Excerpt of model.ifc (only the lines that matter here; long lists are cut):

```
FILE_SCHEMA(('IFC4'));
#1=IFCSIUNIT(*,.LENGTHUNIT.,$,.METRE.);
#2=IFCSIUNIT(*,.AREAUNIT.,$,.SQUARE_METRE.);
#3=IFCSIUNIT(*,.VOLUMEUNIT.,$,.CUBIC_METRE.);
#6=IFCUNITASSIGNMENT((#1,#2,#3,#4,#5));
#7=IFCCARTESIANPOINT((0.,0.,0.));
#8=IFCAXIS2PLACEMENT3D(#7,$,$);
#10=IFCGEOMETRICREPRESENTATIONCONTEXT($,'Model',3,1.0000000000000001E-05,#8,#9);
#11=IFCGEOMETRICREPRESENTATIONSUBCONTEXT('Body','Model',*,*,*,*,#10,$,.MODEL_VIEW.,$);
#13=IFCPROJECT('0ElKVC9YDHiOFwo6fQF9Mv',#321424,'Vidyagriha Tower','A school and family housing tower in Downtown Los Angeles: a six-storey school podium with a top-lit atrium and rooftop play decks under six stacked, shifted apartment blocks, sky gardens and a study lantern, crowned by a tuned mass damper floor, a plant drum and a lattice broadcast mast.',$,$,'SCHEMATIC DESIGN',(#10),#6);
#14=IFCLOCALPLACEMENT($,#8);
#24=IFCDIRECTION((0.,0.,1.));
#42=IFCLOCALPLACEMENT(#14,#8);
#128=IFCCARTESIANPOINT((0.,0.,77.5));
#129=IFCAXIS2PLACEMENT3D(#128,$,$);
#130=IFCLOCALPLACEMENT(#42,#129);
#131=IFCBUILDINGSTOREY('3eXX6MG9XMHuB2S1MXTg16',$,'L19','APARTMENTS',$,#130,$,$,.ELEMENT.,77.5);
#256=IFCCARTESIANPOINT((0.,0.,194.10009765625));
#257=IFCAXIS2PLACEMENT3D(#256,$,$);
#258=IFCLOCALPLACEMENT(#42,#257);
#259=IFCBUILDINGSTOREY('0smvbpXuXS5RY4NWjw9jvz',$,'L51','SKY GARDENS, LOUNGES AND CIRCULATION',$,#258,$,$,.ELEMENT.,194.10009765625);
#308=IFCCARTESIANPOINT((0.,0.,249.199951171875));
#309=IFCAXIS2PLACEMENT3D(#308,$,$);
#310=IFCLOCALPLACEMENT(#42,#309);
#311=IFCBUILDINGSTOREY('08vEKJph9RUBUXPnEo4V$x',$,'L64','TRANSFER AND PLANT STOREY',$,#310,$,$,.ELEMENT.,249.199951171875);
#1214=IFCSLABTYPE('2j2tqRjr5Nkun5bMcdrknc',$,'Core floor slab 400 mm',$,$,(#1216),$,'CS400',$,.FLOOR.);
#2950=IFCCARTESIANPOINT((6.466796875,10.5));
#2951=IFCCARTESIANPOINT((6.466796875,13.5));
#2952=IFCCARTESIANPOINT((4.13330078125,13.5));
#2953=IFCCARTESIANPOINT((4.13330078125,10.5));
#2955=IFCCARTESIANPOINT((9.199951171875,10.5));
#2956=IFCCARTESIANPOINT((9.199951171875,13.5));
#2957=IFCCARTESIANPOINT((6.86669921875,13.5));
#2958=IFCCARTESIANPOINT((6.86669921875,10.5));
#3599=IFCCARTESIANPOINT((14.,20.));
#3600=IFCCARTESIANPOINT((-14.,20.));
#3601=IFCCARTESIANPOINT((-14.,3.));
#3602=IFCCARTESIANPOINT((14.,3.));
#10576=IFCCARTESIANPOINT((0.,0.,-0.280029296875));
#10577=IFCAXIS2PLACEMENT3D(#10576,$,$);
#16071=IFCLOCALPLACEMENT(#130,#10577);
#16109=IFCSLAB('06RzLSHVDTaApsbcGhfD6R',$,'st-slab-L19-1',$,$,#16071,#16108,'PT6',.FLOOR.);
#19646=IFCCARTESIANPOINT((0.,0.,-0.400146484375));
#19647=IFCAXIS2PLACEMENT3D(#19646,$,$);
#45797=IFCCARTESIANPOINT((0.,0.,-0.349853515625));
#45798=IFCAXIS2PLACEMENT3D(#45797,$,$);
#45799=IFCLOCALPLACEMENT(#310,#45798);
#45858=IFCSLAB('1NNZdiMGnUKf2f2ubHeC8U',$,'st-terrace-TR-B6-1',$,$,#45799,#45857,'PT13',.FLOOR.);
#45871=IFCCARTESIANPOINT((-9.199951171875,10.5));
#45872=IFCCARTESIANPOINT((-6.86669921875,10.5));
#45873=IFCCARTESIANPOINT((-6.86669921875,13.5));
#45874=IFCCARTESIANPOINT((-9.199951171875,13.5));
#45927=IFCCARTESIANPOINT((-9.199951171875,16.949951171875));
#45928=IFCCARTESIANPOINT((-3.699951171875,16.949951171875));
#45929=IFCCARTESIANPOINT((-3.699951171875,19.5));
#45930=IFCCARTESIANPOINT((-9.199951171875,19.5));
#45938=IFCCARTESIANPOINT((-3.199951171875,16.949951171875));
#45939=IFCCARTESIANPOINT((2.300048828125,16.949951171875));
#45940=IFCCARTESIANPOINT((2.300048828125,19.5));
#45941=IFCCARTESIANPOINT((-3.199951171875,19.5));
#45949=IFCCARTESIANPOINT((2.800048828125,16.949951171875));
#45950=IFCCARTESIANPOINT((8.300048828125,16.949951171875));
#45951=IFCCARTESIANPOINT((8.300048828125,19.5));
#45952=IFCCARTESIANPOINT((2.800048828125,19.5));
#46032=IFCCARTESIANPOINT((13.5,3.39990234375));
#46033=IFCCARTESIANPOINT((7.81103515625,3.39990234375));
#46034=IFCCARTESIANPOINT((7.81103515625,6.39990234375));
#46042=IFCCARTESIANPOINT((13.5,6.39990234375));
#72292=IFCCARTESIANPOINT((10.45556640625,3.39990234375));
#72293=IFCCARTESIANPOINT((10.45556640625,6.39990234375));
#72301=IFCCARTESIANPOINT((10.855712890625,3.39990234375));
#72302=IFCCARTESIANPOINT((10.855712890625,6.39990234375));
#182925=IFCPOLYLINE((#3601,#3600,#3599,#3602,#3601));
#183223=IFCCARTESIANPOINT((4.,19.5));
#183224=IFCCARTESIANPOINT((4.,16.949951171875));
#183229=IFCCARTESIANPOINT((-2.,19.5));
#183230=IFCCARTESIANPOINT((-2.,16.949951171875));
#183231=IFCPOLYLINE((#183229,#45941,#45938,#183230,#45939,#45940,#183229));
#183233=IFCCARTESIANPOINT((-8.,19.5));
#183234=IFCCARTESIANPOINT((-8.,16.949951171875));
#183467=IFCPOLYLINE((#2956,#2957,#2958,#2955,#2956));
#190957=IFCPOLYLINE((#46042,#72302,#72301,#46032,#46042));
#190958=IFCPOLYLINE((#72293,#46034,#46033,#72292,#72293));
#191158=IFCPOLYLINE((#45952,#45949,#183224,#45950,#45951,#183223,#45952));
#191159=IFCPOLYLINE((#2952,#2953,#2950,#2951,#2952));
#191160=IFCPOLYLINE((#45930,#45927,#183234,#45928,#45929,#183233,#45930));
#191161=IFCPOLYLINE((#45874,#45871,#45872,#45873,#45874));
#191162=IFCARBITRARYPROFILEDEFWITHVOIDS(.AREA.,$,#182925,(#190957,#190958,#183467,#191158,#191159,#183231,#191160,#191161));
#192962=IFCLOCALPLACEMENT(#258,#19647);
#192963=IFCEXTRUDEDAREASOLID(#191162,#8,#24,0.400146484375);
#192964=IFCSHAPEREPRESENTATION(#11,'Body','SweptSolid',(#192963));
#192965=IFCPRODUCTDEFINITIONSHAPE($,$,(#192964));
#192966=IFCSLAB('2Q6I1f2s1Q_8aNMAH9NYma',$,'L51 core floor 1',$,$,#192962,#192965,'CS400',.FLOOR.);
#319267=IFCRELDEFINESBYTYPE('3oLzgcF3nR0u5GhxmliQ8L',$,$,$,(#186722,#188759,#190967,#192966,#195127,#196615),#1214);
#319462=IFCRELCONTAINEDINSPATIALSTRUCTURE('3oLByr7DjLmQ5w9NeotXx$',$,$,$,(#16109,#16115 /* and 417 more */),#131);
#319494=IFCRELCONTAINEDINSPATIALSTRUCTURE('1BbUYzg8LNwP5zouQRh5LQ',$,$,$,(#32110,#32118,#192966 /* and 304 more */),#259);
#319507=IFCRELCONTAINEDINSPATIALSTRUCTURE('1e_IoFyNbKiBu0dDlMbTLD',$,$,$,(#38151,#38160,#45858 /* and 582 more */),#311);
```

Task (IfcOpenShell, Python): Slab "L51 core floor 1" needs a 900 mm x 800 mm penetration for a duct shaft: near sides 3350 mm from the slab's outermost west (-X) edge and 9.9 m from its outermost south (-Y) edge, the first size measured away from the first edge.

```python
import numpy as np
import ifcopenshell
import ifcopenshell.api.feature
import ifcopenshell.api.geometry
import ifcopenshell.api.root
import ifcopenshell.geom
import ifcopenshell.util.placement
import ifcopenshell.util.representation
import ifcopenshell.util.shape
import ifcopenshell.util.unit

model = ifcopenshell.open("model.ifc")
unit_scale = ifcopenshell.util.unit.calculate_unit_scale(model)
settings = ifcopenshell.geom.settings()


def volume(element):
    """Net volume in cubic metres, openings subtracted."""
    shape = ifcopenshell.geom.create_shape(settings, element)
    return ifcopenshell.util.shape.get_volume(shape.geometry)


slab = model.by_id(192966)
before = volume(slab)

# Extent in the slab's own axes, in metres. The edges named are its -X and -Y sides.
slab_shape = ifcopenshell.geom.create_shape(settings, slab)
vertices = ifcopenshell.util.shape.get_vertices(slab_shape.geometry)
x_min, y_min, bottom = vertices.min(axis=0)
top = vertices[:, 2].max()

opening = ifcopenshell.api.root.create_entity(model, ifc_class="IfcOpeningElement", name="Duct shaft opening", predefined_type="OPENING")
context = ifcopenshell.util.representation.get_context(model, "Model", "Body", "MODEL_VIEW")
width, depth = 0.9, 0.8
outline = [(0.0, 0.0), (width, 0.0), (width, depth), (0.0, depth), (0.0, 0.0)]
# Overshoot both faces by 50 mm so the cut is clean.
shape = ifcopenshell.api.geometry.add_slab_representation(
    model, context=context, depth=top - bottom + 0.1, polyline=outline
)
ifcopenshell.api.geometry.assign_representation(model, product=opening, representation=shape)

matrix = ifcopenshell.util.placement.get_local_placement(slab.ObjectPlacement)
matrix[:, 3] = matrix @ np.append(np.array([x_min + 3.35, y_min + 9.9, bottom - 0.05]) / unit_scale, 1.0)
ifcopenshell.api.geometry.edit_object_placement(model, product=opening, matrix=matrix, is_si=False)
ifcopenshell.api.feature.add_feature(model, feature=opening, element=slab)

after = volume(slab)

print(f"slab volume {before:.3f} -> {after:.3f} m3")

model.write("model_updated.ifc")
```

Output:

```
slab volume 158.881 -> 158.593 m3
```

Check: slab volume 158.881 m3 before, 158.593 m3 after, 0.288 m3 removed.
